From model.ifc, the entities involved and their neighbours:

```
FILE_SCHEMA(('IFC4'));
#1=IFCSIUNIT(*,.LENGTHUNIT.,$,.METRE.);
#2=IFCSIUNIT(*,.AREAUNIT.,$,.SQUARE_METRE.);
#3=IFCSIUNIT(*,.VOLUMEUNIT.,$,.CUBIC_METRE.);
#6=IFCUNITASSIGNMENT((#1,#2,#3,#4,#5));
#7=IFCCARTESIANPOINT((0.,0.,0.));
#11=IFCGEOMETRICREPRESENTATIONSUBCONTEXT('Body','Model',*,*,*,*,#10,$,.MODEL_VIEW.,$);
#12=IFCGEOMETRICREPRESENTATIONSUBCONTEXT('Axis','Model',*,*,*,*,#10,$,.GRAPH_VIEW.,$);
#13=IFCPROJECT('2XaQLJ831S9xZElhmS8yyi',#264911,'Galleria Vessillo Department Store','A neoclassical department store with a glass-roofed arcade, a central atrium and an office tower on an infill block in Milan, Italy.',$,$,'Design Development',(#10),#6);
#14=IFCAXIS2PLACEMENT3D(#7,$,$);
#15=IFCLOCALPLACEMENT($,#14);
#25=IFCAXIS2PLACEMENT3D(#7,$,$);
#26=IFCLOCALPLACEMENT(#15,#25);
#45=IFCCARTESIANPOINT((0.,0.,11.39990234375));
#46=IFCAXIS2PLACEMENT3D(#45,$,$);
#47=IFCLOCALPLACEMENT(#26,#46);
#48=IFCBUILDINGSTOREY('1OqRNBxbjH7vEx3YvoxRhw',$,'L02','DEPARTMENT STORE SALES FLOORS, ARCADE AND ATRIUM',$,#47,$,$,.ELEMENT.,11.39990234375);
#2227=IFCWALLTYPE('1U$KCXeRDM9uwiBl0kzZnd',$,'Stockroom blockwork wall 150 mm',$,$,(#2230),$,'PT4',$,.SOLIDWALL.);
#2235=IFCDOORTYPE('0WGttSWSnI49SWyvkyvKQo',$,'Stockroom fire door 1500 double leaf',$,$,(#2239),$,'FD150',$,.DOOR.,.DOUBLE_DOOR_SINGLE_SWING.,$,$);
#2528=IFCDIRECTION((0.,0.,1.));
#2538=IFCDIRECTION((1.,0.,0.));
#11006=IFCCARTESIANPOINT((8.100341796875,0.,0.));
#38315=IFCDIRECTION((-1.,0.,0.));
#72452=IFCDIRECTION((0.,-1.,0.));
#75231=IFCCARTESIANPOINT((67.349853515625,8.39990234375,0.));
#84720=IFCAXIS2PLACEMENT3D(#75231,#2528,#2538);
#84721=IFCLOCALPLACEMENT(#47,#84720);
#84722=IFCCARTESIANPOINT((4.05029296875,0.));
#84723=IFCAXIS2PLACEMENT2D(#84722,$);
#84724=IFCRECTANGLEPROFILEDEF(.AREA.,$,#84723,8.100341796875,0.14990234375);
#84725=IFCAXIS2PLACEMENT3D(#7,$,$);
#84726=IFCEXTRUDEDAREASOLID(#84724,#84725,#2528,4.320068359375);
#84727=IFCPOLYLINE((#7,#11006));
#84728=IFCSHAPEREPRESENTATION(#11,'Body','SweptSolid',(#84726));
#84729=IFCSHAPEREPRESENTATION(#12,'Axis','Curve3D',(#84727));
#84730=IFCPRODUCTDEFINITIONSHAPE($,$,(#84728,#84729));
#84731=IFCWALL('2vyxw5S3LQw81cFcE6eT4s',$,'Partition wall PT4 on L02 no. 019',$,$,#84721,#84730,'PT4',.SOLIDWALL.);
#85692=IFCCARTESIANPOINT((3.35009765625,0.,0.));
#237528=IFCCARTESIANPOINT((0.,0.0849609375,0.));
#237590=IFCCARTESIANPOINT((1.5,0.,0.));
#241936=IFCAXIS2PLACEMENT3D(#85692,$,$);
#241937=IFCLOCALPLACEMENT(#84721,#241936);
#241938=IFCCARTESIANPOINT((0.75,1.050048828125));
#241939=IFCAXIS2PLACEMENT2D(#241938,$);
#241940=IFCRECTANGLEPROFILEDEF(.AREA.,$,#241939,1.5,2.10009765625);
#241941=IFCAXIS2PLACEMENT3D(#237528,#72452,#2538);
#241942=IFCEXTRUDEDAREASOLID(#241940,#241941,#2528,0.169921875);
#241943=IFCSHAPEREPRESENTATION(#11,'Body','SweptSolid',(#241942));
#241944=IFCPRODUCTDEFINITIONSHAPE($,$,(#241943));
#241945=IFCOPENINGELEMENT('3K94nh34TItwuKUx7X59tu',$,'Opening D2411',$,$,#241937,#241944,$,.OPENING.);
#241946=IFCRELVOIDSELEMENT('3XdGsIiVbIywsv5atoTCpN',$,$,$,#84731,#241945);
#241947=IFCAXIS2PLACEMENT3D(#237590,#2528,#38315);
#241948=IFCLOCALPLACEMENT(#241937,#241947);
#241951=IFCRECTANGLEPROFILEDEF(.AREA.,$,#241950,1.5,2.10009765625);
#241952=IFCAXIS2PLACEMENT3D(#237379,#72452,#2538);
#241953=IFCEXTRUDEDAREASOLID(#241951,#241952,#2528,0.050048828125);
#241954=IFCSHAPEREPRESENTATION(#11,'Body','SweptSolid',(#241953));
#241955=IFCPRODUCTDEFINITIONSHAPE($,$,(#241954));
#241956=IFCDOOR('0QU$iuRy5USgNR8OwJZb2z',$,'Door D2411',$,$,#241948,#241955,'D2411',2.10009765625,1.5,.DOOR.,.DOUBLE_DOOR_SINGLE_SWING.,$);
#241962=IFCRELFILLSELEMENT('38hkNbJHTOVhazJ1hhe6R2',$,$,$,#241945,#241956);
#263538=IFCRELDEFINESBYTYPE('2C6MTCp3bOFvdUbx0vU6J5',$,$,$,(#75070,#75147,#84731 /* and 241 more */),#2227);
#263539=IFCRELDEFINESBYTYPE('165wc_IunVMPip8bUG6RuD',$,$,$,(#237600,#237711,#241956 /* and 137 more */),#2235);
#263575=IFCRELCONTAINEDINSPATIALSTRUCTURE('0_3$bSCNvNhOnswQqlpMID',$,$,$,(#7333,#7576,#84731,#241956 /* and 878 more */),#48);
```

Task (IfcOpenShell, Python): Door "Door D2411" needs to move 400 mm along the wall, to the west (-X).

```python
import ifcopenshell
import ifcopenshell.api.geometry
import ifcopenshell.util.placement

model = ifcopenshell.open("model.ifc")

door = model.by_guid("0QU$iuRy5USgNR8OwJZb2z")
opening = door.FillsVoids[0].RelatingOpeningElement
wall = opening.VoidsElements[0].RelatingBuildingElement

wall_matrix = ifcopenshell.util.placement.get_local_placement(wall.ObjectPlacement)
shift = wall_matrix[:3, 0] * -0.4
before = ifcopenshell.util.placement.get_local_placement(door.ObjectPlacement)[:3, 3].copy()

# The door is placed relative to its opening, so it follows when the opening moves.
matrix = ifcopenshell.util.placement.get_local_placement(opening.ObjectPlacement)
matrix[:3, 3] += shift
ifcopenshell.api.geometry.edit_object_placement(
    model, product=opening, matrix=matrix, is_si=False, should_transform_children=True
)

after = ifcopenshell.util.placement.get_local_placement(door.ObjectPlacement)[:3, 3]
print("door moved by", (after - before).round(3) + 0.0)

model.write("model_updated.ifc")
```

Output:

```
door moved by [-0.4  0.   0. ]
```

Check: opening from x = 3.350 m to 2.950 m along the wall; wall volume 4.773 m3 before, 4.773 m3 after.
